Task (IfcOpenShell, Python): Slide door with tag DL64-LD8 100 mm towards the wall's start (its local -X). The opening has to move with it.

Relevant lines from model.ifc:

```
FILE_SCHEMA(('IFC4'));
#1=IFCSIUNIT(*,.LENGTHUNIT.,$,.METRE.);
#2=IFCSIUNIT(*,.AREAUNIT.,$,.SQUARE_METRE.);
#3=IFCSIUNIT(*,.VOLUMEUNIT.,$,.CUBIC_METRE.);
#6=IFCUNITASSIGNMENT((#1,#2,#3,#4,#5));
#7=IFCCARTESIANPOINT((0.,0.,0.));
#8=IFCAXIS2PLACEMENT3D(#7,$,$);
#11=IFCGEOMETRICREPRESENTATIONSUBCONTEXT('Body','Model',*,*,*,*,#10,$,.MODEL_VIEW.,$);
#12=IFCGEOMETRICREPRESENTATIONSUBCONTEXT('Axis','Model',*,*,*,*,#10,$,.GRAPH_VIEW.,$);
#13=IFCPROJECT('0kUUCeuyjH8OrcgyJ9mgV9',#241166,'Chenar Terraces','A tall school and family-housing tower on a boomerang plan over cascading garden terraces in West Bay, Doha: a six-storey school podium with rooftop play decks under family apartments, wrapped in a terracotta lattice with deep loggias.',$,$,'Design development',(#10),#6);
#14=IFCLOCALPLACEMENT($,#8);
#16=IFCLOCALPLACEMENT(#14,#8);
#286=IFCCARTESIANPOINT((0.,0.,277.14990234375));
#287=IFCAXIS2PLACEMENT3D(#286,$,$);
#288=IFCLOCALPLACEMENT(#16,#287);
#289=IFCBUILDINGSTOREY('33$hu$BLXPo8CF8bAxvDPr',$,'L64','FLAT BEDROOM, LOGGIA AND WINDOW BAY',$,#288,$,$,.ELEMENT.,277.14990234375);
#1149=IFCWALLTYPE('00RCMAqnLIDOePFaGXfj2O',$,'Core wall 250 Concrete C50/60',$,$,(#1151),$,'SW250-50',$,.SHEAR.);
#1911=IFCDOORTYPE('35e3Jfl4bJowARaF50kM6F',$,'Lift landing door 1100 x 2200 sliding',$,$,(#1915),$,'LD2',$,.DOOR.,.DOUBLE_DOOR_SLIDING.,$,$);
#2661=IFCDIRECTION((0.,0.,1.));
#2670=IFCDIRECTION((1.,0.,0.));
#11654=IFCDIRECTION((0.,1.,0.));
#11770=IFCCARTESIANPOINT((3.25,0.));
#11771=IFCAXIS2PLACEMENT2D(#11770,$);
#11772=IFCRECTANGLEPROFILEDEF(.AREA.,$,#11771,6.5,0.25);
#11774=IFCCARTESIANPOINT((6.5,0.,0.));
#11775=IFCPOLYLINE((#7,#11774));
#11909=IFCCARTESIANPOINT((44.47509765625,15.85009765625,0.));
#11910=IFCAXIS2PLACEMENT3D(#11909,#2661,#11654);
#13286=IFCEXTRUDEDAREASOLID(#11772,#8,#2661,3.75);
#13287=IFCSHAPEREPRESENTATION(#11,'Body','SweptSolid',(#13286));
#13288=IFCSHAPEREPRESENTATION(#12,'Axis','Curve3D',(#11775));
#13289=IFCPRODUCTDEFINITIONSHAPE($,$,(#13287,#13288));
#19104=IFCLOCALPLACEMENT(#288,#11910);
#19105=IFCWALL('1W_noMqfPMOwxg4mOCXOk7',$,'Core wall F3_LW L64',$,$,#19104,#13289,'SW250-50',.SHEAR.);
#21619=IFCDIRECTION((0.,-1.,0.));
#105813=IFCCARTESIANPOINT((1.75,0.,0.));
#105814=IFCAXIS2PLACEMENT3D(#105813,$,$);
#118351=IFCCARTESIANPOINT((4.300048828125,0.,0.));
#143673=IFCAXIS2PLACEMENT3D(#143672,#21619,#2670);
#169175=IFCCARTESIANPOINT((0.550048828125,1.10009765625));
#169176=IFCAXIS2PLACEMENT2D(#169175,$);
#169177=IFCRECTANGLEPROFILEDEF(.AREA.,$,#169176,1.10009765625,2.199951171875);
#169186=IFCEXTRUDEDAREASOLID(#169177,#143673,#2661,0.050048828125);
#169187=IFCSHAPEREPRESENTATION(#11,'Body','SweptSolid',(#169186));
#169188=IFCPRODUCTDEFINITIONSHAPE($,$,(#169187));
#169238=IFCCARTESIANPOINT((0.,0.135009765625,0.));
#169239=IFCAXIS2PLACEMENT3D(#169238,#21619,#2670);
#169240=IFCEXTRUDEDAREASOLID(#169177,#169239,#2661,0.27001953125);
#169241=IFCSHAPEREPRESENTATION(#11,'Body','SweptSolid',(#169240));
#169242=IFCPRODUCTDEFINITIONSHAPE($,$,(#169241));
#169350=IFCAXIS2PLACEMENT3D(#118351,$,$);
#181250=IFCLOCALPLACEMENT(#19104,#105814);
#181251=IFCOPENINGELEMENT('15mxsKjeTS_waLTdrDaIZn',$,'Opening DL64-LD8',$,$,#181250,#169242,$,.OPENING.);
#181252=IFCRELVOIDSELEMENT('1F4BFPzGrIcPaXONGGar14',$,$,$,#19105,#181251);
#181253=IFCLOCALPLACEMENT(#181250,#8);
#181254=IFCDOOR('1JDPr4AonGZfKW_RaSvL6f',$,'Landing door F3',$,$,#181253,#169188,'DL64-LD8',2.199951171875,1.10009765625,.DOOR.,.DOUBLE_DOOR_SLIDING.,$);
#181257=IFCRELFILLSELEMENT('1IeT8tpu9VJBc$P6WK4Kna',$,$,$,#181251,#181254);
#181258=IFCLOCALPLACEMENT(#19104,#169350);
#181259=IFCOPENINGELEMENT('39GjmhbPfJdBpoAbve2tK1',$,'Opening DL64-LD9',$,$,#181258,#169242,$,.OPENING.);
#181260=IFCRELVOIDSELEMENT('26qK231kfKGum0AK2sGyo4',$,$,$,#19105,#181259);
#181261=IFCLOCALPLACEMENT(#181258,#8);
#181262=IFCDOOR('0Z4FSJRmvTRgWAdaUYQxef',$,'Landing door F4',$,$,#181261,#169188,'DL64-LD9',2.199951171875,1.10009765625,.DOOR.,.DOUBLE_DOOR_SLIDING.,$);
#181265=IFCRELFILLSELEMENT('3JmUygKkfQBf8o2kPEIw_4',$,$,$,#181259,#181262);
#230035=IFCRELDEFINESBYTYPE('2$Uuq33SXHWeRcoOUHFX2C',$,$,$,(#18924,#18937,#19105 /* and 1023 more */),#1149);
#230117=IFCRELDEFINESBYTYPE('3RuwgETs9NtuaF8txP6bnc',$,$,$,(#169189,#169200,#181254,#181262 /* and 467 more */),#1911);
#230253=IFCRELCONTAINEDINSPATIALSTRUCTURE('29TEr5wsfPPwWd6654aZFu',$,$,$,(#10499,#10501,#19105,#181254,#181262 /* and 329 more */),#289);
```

```python
import ifcopenshell
import ifcopenshell.api.geometry
import ifcopenshell.util.placement

model = ifcopenshell.open("model.ifc")

door = model.by_guid("1JDPr4AonGZfKW_RaSvL6f")
opening = door.FillsVoids[0].RelatingOpeningElement
wall = opening.VoidsElements[0].RelatingBuildingElement

wall_matrix = ifcopenshell.util.placement.get_local_placement(wall.ObjectPlacement)
shift = wall_matrix[:3, 0] * -0.1
before = ifcopenshell.util.placement.get_local_placement(door.ObjectPlacement)[:3, 3].copy()

# The door is placed relative to its opening, so it follows when the opening moves.
matrix = ifcopenshell.util.placement.get_local_placement(opening.ObjectPlacement)
matrix[:3, 3] += shift
ifcopenshell.api.geometry.edit_object_placement(
    model, product=opening, matrix=matrix, is_si=False, should_transform_children=True
)

after = ifcopenshell.util.placement.get_local_placement(door.ObjectPlacement)[:3, 3]
print("door moved by", (after - before).round(3) + 0.0)

model.write("model_updated.ifc")
```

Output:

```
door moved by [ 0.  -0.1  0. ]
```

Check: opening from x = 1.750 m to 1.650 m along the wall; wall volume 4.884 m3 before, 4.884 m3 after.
